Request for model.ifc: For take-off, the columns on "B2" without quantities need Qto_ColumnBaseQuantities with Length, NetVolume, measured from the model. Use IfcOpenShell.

First a look at what the model holds.

```python
import ifcopenshell
import ifcopenshell.util.element
import ifcopenshell.util.unit

model = ifcopenshell.open("model.ifc")
print(model.schema)
for unit_type in ("LENGTHUNIT", "AREAUNIT", "VOLUMEUNIT"):
    print(unit_type, ifcopenshell.util.unit.calculate_unit_scale(model, unit_type))
storey = next(s for s in model.by_type("IfcBuildingStorey") if s.Name == "B2")
columns = [e for e in ifcopenshell.util.element.get_decomposition(storey) if e.is_a("IfcColumn")]
for e in sorted(columns, key=lambda e: e.id()):
    print(e.id(), e.is_a(), e.Name, list(ifcopenshell.util.element.get_psets(e, qtos_only=True)), sep=" | ")
```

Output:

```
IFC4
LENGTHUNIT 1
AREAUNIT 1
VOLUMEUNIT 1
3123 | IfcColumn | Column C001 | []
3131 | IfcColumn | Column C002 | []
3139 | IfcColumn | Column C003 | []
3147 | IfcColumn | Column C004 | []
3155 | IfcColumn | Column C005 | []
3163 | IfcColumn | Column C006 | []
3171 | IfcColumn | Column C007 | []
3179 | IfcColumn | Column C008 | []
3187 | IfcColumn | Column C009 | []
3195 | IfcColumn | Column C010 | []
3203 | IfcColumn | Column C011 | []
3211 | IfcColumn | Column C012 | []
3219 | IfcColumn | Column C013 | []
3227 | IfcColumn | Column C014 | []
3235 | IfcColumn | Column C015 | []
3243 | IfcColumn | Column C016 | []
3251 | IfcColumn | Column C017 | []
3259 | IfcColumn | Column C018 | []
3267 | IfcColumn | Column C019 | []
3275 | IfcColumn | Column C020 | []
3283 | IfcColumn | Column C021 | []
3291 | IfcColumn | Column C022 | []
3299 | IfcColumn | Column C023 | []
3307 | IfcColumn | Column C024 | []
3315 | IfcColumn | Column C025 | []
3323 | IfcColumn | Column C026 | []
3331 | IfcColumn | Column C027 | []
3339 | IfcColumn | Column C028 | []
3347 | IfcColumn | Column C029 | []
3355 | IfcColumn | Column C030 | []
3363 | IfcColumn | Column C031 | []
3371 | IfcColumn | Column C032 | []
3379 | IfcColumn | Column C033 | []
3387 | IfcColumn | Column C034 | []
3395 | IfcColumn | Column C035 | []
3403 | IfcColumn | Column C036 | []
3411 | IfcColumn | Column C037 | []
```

```python
import ifcopenshell
import ifcopenshell.api.pset
import ifcopenshell.geom
import ifcopenshell.util.element
import ifcopenshell.util.shape
import ifcopenshell.util.unit

model = ifcopenshell.open("model.ifc")
unit_scale = ifcopenshell.util.unit.calculate_unit_scale(model)
volume_scale = ifcopenshell.util.unit.calculate_unit_scale(model, "VOLUMEUNIT")
settings = ifcopenshell.geom.settings()

storey = next(s for s in model.by_type("IfcBuildingStorey") if s.Name == "B2")
columns = [e for e in ifcopenshell.util.element.get_decomposition(storey) if e.is_a("IfcColumn")]

for e in sorted(columns, key=lambda e: e.id()):
    if ifcopenshell.util.element.get_psets(e, qtos_only=True, should_inherit=False):
        continue
    # Geometry comes back in metres, in the element's own axes.
    shape = ifcopenshell.geom.create_shape(settings, e)
    values = {
        "Length": ifcopenshell.util.shape.get_z(shape.geometry) / unit_scale,
        "NetVolume": ifcopenshell.util.shape.get_volume(shape.geometry) / volume_scale,
    }
    qto = ifcopenshell.api.pset.add_qto(model, product=e, name="Qto_ColumnBaseQuantities")
    ifcopenshell.api.pset.edit_qto(model, qto=qto, properties=values)
    print(e.id(), {k: round(v, 3) for k, v in values.items()})

model.write("model-out.ifc")
```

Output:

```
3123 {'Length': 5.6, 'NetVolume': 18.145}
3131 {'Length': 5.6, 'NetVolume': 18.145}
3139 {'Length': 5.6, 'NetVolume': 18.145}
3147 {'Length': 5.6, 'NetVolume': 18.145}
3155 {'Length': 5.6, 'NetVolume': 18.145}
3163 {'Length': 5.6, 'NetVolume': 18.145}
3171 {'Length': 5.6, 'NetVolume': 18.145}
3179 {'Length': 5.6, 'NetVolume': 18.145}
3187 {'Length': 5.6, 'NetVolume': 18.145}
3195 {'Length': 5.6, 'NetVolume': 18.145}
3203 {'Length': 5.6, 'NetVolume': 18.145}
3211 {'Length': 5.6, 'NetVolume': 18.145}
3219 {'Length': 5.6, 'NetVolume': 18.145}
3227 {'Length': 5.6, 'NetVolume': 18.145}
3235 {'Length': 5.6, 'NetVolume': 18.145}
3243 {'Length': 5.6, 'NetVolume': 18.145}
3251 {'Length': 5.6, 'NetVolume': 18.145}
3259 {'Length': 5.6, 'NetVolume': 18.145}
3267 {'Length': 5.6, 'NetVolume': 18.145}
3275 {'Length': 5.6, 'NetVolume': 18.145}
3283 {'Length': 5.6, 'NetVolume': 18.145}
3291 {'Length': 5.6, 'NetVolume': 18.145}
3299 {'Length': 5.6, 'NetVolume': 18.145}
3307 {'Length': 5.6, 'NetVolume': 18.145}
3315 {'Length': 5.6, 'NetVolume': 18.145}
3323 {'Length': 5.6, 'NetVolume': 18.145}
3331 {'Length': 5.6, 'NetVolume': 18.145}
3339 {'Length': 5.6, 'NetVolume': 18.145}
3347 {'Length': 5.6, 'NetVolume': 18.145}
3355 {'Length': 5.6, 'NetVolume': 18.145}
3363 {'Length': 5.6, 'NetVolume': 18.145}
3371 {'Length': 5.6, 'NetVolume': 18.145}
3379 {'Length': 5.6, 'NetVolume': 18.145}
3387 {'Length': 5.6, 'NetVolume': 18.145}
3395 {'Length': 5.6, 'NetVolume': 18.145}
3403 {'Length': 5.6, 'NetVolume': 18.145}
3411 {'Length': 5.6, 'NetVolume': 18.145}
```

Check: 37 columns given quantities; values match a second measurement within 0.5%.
